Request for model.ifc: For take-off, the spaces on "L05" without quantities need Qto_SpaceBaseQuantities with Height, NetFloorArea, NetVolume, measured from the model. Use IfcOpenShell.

First a look at what the model holds.

```python
import ifcopenshell
import ifcopenshell.util.element
import ifcopenshell.util.unit

model = ifcopenshell.open("model.ifc")
print(model.schema)
for unit_type in ("LENGTHUNIT", "AREAUNIT", "VOLUMEUNIT"):
    print(unit_type, ifcopenshell.util.unit.calculate_unit_scale(model, unit_type))
storey = next(s for s in model.by_type("IfcBuildingStorey") if s.Name == "L05")
spaces = [e for e in ifcopenshell.util.element.get_decomposition(storey) if e.is_a("IfcSpace")]
for e in sorted(spaces, key=lambda e: e.id()):
    print(e.id(), e.is_a(), e.Name, list(ifcopenshell.util.element.get_psets(e, qtos_only=True)), sep=" | ")
```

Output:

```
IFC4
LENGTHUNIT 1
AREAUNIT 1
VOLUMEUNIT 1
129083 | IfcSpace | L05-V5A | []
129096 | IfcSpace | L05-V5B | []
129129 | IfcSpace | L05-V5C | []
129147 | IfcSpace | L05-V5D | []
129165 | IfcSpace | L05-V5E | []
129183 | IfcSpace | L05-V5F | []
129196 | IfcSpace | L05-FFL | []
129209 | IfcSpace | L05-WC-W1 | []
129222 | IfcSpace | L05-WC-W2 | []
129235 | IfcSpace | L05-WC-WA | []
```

```python
import ifcopenshell
import ifcopenshell.api.pset
import ifcopenshell.geom
import ifcopenshell.util.element
import ifcopenshell.util.shape
import ifcopenshell.util.unit

model = ifcopenshell.open("model.ifc")
unit_scale = ifcopenshell.util.unit.calculate_unit_scale(model)
area_scale = ifcopenshell.util.unit.calculate_unit_scale(model, "AREAUNIT")
volume_scale = ifcopenshell.util.unit.calculate_unit_scale(model, "VOLUMEUNIT")
settings = ifcopenshell.geom.settings()

storey = next(s for s in model.by_type("IfcBuildingStorey") if s.Name == "L05")
spaces = [e for e in ifcopenshell.util.element.get_decomposition(storey) if e.is_a("IfcSpace")]

for e in sorted(spaces, key=lambda e: e.id()):
    if ifcopenshell.util.element.get_psets(e, qtos_only=True, should_inherit=False):
        continue
    # Geometry comes back in metres, in the element's own axes.
    shape = ifcopenshell.geom.create_shape(settings, e)
    values = {
        "Height": ifcopenshell.util.shape.get_z(shape.geometry) / unit_scale,
        "NetFloorArea": ifcopenshell.util.shape.get_footprint_area(shape.geometry) / area_scale,
        "NetVolume": ifcopenshell.util.shape.get_volume(shape.geometry) / volume_scale,
    }
    qto = ifcopenshell.api.pset.add_qto(model, product=e, name="Qto_SpaceBaseQuantities")
    ifcopenshell.api.pset.edit_qto(model, qto=qto, properties=values)
    print(e.id(), {k: round(v, 3) for k, v in values.items()})

model.write("model_edited.ifc")
```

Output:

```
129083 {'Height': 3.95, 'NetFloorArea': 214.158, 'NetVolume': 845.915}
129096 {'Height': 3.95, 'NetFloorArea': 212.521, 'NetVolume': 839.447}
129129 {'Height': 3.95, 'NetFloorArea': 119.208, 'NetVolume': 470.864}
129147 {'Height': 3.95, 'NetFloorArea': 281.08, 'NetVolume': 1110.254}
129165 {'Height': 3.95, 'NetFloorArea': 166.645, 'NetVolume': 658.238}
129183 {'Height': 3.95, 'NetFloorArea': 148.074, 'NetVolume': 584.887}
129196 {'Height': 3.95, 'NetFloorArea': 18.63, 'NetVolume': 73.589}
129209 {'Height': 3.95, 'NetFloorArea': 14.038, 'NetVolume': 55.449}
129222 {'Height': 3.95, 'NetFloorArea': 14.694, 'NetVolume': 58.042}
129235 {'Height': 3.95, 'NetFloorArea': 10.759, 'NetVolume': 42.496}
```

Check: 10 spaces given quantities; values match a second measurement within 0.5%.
